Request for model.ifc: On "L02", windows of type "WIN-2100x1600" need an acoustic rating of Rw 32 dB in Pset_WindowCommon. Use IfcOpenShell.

First a look at what the model holds.

```python
import ifcopenshell
import ifcopenshell.util.element

model = ifcopenshell.open("model.ifc")
print(model.schema)
storey = next(s for s in model.by_type("IfcBuildingStorey") if s.Name == "L02")
windows = [e for e in ifcopenshell.util.element.get_decomposition(storey) if e.is_a("IfcWindow")]
seen = {}
for e in windows:
    element_type = ifcopenshell.util.element.get_type(e)
    key = (element_type.Name if element_type != e and element_type else None, ifcopenshell.util.element.get_pset(e, "Pset_WindowCommon", "AcousticRating"))
    seen[key] = seen.get(key, 0) + 1
for (name, value), count in sorted(seen.items(), key=str):
    print(count, "x", name, "|", value)
```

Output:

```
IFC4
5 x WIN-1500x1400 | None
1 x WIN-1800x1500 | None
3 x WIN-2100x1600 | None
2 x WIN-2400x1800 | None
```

```python
import ifcopenshell
import ifcopenshell.api.pset
import ifcopenshell.util.element

model = ifcopenshell.open("model.ifc")

storey = next(s for s in model.by_type("IfcBuildingStorey") if s.Name == "L02")
windows = [e for e in ifcopenshell.util.element.get_decomposition(storey) if e.is_a("IfcWindow")]

count = 0
for e in windows:
    element_type = ifcopenshell.util.element.get_type(e)
    if element_type in (None, e) or element_type.Name != "WIN-2100x1600":
        continue
    # add_pset returns the element's existing set when there is one.
    pset = ifcopenshell.api.pset.add_pset(model, product=e, name="Pset_WindowCommon")
    ifcopenshell.api.pset.edit_pset(model, pset=pset, properties={"AcousticRating": "Rw 32 dB"})
    count += 1

print(count, "windows updated")

model.write("model-out.ifc")
```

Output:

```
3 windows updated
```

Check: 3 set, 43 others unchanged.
